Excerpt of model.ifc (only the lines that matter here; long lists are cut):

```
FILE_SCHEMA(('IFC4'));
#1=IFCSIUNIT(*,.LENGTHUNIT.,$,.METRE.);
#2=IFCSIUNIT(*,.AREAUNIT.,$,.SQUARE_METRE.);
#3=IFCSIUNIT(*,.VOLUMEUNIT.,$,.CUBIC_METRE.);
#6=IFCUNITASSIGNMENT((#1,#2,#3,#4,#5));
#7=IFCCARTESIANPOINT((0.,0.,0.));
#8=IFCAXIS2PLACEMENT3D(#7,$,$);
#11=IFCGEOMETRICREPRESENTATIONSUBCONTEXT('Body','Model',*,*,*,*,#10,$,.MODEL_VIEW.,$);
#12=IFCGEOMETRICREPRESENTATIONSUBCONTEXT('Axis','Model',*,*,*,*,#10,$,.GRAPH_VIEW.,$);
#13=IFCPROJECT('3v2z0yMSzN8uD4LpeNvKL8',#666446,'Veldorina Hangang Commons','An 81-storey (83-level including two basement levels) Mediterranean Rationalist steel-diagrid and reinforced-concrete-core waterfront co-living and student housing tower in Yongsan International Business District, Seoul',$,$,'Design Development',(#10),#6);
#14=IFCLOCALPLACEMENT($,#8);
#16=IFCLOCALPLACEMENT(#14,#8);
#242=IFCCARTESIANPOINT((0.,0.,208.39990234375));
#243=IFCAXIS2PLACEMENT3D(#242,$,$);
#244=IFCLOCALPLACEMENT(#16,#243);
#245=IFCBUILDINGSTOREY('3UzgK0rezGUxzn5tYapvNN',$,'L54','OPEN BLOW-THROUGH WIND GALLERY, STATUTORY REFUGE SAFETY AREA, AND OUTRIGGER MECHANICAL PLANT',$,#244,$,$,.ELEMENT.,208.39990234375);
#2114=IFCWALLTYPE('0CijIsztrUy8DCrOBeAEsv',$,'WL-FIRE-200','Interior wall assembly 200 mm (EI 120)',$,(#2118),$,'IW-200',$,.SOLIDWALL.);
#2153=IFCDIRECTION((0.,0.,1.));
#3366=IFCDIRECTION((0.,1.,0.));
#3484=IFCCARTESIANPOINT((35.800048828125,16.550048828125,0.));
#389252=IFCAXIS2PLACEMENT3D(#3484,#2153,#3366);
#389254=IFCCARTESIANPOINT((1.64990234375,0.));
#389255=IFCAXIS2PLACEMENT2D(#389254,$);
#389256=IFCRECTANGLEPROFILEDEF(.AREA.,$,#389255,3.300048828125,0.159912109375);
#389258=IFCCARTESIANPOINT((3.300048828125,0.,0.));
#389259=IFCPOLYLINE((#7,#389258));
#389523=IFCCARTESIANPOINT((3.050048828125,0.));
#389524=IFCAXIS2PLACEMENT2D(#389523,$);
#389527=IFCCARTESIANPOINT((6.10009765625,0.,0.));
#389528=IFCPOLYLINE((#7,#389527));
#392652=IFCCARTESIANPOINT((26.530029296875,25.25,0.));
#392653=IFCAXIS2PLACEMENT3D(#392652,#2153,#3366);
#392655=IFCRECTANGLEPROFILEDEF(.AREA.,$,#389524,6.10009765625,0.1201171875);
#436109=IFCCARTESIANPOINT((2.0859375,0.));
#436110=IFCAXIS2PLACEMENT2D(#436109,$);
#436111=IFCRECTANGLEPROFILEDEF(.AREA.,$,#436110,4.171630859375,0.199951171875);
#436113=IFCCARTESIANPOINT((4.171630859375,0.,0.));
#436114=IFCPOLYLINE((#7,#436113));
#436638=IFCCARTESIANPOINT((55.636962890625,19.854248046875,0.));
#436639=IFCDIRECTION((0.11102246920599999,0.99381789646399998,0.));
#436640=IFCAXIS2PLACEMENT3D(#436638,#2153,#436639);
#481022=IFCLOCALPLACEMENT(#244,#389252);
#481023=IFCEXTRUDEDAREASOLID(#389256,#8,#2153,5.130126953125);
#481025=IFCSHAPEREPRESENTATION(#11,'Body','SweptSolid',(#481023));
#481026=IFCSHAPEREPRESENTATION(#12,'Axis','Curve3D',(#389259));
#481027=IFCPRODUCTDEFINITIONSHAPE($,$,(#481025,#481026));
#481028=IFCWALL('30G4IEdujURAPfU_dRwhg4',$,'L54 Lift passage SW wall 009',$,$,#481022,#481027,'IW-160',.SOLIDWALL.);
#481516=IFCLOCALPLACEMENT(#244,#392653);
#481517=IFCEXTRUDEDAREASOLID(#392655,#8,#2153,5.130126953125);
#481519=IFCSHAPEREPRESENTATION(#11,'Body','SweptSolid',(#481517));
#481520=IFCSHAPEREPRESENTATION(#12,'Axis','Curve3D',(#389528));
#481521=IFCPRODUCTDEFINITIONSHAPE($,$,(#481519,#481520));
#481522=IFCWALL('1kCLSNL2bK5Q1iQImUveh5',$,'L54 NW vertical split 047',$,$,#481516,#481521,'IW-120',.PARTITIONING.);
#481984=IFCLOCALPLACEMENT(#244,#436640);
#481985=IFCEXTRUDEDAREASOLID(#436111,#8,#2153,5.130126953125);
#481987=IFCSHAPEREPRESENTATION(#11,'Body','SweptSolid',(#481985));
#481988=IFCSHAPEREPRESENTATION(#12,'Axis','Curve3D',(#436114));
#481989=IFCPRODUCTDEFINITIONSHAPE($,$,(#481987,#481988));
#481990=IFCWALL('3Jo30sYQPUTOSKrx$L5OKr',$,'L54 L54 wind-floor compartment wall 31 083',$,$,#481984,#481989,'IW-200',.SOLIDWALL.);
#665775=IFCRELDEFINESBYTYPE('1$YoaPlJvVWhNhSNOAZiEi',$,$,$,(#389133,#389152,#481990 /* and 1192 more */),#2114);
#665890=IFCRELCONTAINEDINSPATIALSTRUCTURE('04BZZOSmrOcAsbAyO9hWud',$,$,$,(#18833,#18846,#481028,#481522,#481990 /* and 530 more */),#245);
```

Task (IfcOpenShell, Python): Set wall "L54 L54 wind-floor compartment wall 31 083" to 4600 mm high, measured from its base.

```python
import ifcopenshell
import ifcopenshell.geom
import ifcopenshell.util.representation
import ifcopenshell.util.shape
import ifcopenshell.util.unit

model = ifcopenshell.open("model.ifc")
unit_scale = ifcopenshell.util.unit.calculate_unit_scale(model)
settings = ifcopenshell.geom.settings()


def volume(element):
    """Net volume in cubic metres, openings subtracted."""
    shape = ifcopenshell.geom.create_shape(settings, element)
    return ifcopenshell.util.shape.get_volume(shape.geometry)


wall = model.by_guid("3Jo30sYQPUTOSKrx$L5OKr")
before = volume(wall)

body = ifcopenshell.util.representation.get_representation(wall, "Model", "Body")
solid = body.Items[0]
old_height = solid.Depth
solid.Depth = 4.6 / unit_scale
after = volume(wall)

print(f"height {old_height:g} -> {solid.Depth:g}, volume {before:.3f} -> {after:.3f} m3")

model.write("model_rev.ifc")
```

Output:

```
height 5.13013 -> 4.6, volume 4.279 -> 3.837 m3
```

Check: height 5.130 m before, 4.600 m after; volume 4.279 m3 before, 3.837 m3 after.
